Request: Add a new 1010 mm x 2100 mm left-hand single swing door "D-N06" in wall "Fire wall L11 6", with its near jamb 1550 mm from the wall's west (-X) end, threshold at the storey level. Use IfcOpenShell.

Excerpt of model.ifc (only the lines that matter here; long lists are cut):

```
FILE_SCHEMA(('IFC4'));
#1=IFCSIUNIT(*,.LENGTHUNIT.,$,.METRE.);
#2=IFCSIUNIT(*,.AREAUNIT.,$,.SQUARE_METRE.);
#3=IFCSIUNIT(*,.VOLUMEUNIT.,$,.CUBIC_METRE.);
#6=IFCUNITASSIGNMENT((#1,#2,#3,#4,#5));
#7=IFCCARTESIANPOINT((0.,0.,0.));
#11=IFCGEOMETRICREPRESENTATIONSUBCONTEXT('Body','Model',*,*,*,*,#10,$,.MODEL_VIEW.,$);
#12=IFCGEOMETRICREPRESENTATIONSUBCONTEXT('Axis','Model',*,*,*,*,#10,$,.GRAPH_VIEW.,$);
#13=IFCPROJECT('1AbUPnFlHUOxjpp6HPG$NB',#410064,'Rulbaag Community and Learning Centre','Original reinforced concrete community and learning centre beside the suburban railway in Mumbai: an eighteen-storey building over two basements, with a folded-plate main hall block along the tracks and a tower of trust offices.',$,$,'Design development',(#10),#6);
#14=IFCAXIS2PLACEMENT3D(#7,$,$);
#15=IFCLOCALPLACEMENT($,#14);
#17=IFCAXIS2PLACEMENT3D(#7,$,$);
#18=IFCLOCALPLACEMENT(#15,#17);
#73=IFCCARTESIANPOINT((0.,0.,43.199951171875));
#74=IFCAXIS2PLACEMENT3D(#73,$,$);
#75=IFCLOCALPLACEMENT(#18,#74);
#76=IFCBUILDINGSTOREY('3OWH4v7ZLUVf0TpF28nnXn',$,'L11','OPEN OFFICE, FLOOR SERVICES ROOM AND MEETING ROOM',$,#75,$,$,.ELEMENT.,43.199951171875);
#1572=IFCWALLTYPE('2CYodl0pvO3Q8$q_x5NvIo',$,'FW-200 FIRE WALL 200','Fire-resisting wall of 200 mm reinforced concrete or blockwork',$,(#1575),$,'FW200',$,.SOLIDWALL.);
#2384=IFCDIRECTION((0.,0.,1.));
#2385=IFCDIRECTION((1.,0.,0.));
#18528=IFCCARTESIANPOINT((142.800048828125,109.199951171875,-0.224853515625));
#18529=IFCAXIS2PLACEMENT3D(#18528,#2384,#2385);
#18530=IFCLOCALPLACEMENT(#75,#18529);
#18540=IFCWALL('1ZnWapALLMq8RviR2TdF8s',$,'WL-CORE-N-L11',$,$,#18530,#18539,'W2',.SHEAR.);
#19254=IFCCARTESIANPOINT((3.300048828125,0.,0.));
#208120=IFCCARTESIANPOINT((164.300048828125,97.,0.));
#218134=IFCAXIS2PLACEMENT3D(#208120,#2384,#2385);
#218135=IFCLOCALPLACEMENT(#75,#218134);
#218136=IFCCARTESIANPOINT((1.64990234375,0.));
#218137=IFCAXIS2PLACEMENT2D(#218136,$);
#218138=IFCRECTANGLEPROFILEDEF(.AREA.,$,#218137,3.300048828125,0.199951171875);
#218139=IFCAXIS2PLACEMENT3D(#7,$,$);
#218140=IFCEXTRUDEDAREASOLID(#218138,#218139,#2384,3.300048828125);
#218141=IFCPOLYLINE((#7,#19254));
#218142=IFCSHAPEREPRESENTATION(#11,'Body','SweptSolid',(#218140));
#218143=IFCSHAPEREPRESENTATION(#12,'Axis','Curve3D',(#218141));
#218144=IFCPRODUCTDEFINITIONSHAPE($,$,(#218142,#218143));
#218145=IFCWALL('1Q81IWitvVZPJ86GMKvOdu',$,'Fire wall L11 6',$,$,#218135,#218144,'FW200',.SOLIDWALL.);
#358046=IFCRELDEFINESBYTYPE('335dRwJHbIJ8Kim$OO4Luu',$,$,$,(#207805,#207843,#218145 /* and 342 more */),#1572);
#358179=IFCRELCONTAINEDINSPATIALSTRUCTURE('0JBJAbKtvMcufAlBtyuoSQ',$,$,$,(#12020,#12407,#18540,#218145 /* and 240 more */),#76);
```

```python
import numpy as np
import ifcopenshell
import ifcopenshell.api.feature
import ifcopenshell.api.geometry
import ifcopenshell.api.root
import ifcopenshell.api.spatial
import ifcopenshell.geom
import ifcopenshell.util.element
import ifcopenshell.util.placement
import ifcopenshell.util.representation
import ifcopenshell.util.shape
import ifcopenshell.util.unit

model = ifcopenshell.open("model.ifc")
unit_scale = ifcopenshell.util.unit.calculate_unit_scale(model)
settings = ifcopenshell.geom.settings()


def volume(element):
    """Net volume in cubic metres, openings subtracted."""
    shape = ifcopenshell.geom.create_shape(settings, element)
    return ifcopenshell.util.shape.get_volume(shape.geometry)


wall = model.by_guid("1Q81IWitvVZPJ86GMKvOdu")
storey = ifcopenshell.util.element.get_container(wall, ifc_class="IfcBuildingStorey")
context = ifcopenshell.util.representation.get_context(model, "Model", "Body", "MODEL_VIEW")
before = volume(wall)

width, height, from_end, sill = 1.01, 2.1, 1.55, 0.0  # metres

# The wall runs along its own X axis, and the end named is its -X end.
wall_shape = ifcopenshell.geom.create_shape(settings, wall)
x, y, z = ifcopenshell.util.shape.get_vertices(wall_shape.geometry).T
start = x.min() + from_end
face, thickness = float(y.min()), float(y.max() - y.min())
wall_matrix = ifcopenshell.util.placement.get_local_placement(wall.ObjectPlacement)
level = ifcopenshell.util.placement.get_local_placement(storey.ObjectPlacement)[2, 3]


def in_wall(x, y):
    """Placement at x, y metres in the wall's axes, at sill height."""
    matrix = wall_matrix.copy()
    matrix[:, 3] = wall_matrix @ np.array([x / unit_scale, y / unit_scale, 0.0, 1.0])
    matrix[2, 3] = level + sill / unit_scale
    return matrix


# Opening: a box that overshoots both wall faces by 50 mm.
opening = ifcopenshell.api.root.create_entity(model, ifc_class="IfcOpeningElement", predefined_type="OPENING")
box = ifcopenshell.api.geometry.add_wall_representation(
    model, context=context, length=width, height=height, thickness=thickness + 0.1
)
ifcopenshell.api.geometry.assign_representation(model, product=opening, representation=box)
ifcopenshell.api.geometry.edit_object_placement(model, product=opening, matrix=in_wall(start, face - 0.05), is_si=False)
ifcopenshell.api.feature.add_feature(model, feature=opening, element=wall)

door = ifcopenshell.api.root.create_entity(model, ifc_class="IfcDoor", name="D-N06", predefined_type="DOOR")
door.OverallWidth, door.OverallHeight = width / unit_scale, height / unit_scale
door.OperationType = "SINGLE_SWING_LEFT"
body = ifcopenshell.api.geometry.add_door_representation(
    model,
    context=context,
    overall_width=door.OverallWidth,
    overall_height=door.OverallHeight,
    operation_type="SINGLE_SWING_LEFT",
    lining_properties={"LiningDepth": thickness / unit_scale, "ThresholdDepth": thickness / unit_scale},
)
ifcopenshell.api.geometry.assign_representation(model, product=door, representation=body)
ifcopenshell.api.spatial.assign_container(model, products=[door], relating_structure=storey)
ifcopenshell.api.feature.add_filling(model, opening=opening, element=door)

# The lining spans the wall, so the door starts at the wall face.
ifcopenshell.api.geometry.edit_object_placement(model, product=door, matrix=in_wall(start, face), is_si=False)

after = volume(wall)

print(f"wall volume {before:.3f} -> {after:.3f} m3")

model.write("model_v2.ifc")
```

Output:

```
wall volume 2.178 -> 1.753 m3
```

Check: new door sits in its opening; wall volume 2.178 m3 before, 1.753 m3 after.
